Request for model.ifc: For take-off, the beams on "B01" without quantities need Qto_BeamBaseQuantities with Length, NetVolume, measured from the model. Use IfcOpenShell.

First a look at what the model holds.

```python
import ifcopenshell
import ifcopenshell.util.element
import ifcopenshell.util.unit

model = ifcopenshell.open("model.ifc")
print(model.schema)
for unit_type in ("LENGTHUNIT", "AREAUNIT", "VOLUMEUNIT"):
    print(unit_type, ifcopenshell.util.unit.calculate_unit_scale(model, unit_type))
storey = next(s for s in model.by_type("IfcBuildingStorey") if s.Name == "B01")
beams = [e for e in ifcopenshell.util.element.get_decomposition(storey) if e.is_a("IfcBeam")]
for e in sorted(beams, key=lambda e: e.id()):
    print(e.id(), e.is_a(), e.Name, list(ifcopenshell.util.element.get_psets(e, qtos_only=True)), sep=" | ")
```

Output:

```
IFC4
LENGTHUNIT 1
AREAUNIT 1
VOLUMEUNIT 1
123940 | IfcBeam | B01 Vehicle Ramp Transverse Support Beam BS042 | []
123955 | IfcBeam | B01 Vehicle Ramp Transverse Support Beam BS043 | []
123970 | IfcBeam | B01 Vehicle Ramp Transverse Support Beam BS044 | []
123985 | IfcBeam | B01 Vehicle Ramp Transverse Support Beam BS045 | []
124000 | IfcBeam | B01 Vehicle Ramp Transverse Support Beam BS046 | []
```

```python
import ifcopenshell
import ifcopenshell.api.pset
import ifcopenshell.geom
import ifcopenshell.util.element
import ifcopenshell.util.shape
import ifcopenshell.util.unit

model = ifcopenshell.open("model.ifc")
unit_scale = ifcopenshell.util.unit.calculate_unit_scale(model)
volume_scale = ifcopenshell.util.unit.calculate_unit_scale(model, "VOLUMEUNIT")
settings = ifcopenshell.geom.settings()

storey = next(s for s in model.by_type("IfcBuildingStorey") if s.Name == "B01")
beams = [e for e in ifcopenshell.util.element.get_decomposition(storey) if e.is_a("IfcBeam")]

for e in sorted(beams, key=lambda e: e.id()):
    if ifcopenshell.util.element.get_psets(e, qtos_only=True, should_inherit=False):
        continue
    # Geometry comes back in metres, in the element's own axes.
    shape = ifcopenshell.geom.create_shape(settings, e)
    values = {
        "Length": ifcopenshell.util.shape.get_max_xyz(shape.geometry) / unit_scale,
        "NetVolume": ifcopenshell.util.shape.get_volume(shape.geometry) / volume_scale,
    }
    qto = ifcopenshell.api.pset.add_qto(model, product=e, name="Qto_BeamBaseQuantities")
    ifcopenshell.api.pset.edit_qto(model, qto=qto, properties=values)
    print(e.id(), {k: round(v, 3) for k, v in values.items()})

model.write("model_v2.ifc")
```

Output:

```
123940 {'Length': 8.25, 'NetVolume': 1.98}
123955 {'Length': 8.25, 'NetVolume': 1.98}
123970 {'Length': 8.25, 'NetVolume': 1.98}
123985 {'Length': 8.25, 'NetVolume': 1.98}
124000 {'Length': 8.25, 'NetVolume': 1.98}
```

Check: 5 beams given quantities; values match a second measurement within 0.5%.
